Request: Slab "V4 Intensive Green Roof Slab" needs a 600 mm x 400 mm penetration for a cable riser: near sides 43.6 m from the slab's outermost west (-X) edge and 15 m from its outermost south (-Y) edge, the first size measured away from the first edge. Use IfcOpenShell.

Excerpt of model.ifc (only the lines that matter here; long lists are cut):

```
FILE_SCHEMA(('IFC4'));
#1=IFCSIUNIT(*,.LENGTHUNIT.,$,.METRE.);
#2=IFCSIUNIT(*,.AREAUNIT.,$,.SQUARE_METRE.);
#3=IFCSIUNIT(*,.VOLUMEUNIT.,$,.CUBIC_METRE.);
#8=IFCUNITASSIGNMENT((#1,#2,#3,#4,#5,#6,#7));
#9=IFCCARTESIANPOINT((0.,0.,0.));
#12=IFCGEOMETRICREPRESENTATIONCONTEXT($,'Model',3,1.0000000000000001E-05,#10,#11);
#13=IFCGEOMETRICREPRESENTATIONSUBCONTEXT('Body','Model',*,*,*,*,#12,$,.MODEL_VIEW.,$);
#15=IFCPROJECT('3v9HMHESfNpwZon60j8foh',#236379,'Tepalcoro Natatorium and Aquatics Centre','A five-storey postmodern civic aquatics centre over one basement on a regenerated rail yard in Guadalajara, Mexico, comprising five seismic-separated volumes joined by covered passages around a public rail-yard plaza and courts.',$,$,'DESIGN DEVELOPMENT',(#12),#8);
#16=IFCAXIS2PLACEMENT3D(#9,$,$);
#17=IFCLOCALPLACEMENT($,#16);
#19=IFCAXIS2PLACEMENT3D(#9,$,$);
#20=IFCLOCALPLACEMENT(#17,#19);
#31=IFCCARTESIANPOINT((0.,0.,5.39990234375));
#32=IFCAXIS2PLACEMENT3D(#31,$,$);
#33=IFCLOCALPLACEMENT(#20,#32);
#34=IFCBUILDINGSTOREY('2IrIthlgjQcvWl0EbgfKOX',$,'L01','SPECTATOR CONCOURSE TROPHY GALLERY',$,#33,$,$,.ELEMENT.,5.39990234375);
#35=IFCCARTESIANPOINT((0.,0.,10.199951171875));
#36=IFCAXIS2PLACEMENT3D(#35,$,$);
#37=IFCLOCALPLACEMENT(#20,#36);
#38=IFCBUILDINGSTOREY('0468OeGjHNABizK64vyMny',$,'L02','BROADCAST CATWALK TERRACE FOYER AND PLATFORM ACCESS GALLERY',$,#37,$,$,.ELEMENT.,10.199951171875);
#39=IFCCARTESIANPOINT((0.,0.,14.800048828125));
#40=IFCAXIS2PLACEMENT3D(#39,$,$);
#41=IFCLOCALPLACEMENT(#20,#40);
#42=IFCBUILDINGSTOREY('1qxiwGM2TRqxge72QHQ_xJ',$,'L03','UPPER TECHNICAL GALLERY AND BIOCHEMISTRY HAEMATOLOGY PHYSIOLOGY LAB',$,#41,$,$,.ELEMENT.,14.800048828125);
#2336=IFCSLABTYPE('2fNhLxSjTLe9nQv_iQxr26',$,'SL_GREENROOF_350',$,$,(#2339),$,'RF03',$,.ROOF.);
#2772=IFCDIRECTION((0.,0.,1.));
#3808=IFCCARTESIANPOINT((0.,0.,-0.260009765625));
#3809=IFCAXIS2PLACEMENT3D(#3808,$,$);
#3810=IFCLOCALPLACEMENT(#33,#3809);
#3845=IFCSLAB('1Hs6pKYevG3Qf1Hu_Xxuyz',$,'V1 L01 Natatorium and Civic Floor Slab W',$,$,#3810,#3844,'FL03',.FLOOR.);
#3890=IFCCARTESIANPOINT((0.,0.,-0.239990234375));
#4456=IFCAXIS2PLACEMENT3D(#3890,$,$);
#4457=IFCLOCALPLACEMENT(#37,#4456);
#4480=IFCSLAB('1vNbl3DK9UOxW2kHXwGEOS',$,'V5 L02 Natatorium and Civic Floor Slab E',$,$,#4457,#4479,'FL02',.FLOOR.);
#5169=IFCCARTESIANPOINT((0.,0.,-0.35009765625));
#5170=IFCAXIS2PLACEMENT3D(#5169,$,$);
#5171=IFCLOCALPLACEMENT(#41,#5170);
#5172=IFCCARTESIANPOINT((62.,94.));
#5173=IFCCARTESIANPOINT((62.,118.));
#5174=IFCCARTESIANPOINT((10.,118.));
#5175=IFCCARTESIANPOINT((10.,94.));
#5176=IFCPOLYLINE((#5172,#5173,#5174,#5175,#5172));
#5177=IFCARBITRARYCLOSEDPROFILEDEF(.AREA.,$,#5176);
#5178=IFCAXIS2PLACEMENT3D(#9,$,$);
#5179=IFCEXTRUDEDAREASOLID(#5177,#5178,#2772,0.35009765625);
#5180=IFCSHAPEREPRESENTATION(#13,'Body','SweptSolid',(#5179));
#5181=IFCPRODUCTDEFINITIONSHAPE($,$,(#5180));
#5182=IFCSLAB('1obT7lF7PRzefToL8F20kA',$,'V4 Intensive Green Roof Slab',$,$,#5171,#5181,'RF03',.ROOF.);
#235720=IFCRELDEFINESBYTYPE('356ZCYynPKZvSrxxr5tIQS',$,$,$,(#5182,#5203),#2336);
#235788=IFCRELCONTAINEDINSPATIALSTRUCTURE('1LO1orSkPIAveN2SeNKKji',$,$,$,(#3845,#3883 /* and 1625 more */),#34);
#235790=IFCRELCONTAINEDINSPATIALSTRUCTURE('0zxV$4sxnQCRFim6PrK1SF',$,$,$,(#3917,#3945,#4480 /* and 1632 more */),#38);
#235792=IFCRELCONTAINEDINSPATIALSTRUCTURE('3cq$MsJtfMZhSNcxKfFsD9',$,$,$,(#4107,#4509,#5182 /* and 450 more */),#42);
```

```python
import numpy as np
import ifcopenshell
import ifcopenshell.api.feature
import ifcopenshell.api.geometry
import ifcopenshell.api.root
import ifcopenshell.geom
import ifcopenshell.util.placement
import ifcopenshell.util.representation
import ifcopenshell.util.shape
import ifcopenshell.util.unit

model = ifcopenshell.open("model.ifc")
unit_scale = ifcopenshell.util.unit.calculate_unit_scale(model)
settings = ifcopenshell.geom.settings()


def volume(element):
    """Net volume in cubic metres, openings subtracted."""
    shape = ifcopenshell.geom.create_shape(settings, element)
    return ifcopenshell.util.shape.get_volume(shape.geometry)


slab = model.by_guid("1obT7lF7PRzefToL8F20kA")
before = volume(slab)

# Extent in the slab's own axes, in metres. The edges named are its -X and -Y sides.
slab_shape = ifcopenshell.geom.create_shape(settings, slab)
vertices = ifcopenshell.util.shape.get_vertices(slab_shape.geometry)
x_min, y_min, bottom = vertices.min(axis=0)
top = vertices[:, 2].max()

opening = ifcopenshell.api.root.create_entity(model, ifc_class="IfcOpeningElement", name="Cable riser opening", predefined_type="OPENING")
context = ifcopenshell.util.representation.get_context(model, "Model", "Body", "MODEL_VIEW")
width, depth = 0.6, 0.4
outline = [(0.0, 0.0), (width, 0.0), (width, depth), (0.0, depth), (0.0, 0.0)]
# Overshoot both faces by 50 mm so the cut is clean.
shape = ifcopenshell.api.geometry.add_slab_representation(
    model, context=context, depth=top - bottom + 0.1, polyline=outline
)
ifcopenshell.api.geometry.assign_representation(model, product=opening, representation=shape)

matrix = ifcopenshell.util.placement.get_local_placement(slab.ObjectPlacement)
matrix[:, 3] = matrix @ np.append(np.array([x_min + 43.6, y_min + 15, bottom - 0.05]) / unit_scale, 1.0)
ifcopenshell.api.geometry.edit_object_placement(model, product=opening, matrix=matrix, is_si=False)
ifcopenshell.api.feature.add_feature(model, feature=opening, element=slab)

after = volume(slab)

print(f"slab volume {before:.3f} -> {after:.3f} m3")

model.write("model_updated.ifc")
```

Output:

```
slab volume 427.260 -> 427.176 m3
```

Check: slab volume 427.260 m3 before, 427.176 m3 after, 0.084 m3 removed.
